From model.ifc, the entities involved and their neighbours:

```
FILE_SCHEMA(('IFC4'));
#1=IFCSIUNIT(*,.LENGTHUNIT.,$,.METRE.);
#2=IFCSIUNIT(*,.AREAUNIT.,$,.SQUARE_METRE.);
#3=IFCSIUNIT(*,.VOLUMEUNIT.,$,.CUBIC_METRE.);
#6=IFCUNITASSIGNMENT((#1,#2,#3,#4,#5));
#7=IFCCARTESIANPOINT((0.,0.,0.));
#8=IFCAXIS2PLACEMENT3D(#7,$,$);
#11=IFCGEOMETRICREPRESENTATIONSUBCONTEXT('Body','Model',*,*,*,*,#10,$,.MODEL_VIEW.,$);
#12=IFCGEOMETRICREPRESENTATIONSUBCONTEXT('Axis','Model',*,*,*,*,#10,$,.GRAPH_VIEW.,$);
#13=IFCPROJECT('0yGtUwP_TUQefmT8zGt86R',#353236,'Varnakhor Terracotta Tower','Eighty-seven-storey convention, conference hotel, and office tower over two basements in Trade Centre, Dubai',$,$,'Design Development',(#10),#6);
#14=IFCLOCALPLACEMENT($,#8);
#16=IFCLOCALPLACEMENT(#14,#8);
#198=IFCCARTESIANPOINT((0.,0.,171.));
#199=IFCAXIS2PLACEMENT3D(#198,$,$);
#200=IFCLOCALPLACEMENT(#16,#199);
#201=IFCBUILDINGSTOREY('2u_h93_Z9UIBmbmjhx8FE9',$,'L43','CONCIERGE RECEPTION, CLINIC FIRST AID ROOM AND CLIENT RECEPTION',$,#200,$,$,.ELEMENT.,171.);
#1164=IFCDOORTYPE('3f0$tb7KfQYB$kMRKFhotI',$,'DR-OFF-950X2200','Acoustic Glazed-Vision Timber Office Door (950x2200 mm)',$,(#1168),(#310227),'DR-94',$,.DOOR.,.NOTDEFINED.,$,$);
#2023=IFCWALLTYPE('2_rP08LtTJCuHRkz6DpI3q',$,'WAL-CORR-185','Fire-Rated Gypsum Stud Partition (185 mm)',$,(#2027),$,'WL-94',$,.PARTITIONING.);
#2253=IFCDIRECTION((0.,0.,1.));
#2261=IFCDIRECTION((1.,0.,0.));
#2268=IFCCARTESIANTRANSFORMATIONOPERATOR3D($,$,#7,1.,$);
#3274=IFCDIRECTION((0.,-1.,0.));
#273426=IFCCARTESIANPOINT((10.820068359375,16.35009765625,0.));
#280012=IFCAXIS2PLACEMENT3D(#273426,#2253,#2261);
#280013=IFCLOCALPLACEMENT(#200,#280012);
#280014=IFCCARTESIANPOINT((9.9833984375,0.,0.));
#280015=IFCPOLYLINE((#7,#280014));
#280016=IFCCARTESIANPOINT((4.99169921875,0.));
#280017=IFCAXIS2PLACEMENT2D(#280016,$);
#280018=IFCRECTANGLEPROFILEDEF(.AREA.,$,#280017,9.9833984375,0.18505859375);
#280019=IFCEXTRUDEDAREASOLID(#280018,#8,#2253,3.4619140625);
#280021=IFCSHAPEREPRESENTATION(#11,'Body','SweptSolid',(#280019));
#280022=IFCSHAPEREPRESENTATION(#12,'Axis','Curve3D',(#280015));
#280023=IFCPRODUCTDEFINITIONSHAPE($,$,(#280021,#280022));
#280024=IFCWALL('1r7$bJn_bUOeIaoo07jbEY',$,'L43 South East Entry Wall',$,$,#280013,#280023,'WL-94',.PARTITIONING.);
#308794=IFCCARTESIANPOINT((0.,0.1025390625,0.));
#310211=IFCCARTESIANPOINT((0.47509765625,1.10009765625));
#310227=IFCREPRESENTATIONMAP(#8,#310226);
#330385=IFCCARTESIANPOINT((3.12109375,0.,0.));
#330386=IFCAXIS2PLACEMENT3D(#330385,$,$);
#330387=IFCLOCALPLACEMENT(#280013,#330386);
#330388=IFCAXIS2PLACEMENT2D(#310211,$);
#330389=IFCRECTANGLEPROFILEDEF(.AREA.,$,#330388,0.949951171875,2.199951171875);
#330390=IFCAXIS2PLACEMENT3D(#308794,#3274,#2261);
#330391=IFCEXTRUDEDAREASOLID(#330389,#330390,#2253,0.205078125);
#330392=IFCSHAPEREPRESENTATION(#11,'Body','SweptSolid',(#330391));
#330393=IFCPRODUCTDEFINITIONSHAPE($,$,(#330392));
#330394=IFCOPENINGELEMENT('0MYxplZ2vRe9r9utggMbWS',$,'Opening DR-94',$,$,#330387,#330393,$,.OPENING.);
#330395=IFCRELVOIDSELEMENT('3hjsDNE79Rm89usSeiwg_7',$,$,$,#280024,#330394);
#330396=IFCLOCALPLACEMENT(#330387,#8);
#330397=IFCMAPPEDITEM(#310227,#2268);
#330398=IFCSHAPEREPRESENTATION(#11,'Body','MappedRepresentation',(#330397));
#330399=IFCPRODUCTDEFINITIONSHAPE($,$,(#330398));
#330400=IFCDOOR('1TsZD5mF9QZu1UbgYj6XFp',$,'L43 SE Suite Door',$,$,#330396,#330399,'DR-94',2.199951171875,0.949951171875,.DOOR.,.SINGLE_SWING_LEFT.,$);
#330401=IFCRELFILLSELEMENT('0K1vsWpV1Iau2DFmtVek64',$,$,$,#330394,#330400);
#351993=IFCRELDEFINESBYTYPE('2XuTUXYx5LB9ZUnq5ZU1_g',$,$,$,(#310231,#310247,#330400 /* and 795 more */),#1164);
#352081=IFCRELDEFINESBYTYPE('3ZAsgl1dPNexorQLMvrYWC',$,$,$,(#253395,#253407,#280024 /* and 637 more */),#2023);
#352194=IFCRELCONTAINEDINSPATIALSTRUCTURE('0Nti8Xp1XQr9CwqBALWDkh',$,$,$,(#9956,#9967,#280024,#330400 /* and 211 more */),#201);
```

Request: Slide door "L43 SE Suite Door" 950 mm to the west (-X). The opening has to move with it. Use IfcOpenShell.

```python
import ifcopenshell
import ifcopenshell.api.geometry
import ifcopenshell.util.placement
import ifcopenshell.util.unit

model = ifcopenshell.open("model.ifc")
unit_scale = ifcopenshell.util.unit.calculate_unit_scale(model)

door = model.by_guid("1TsZD5mF9QZu1UbgYj6XFp")
opening = door.FillsVoids[0].RelatingOpeningElement
wall = opening.VoidsElements[0].RelatingBuildingElement

wall_matrix = ifcopenshell.util.placement.get_local_placement(wall.ObjectPlacement)
shift = wall_matrix[:3, 0] * -0.95 / unit_scale
before = ifcopenshell.util.placement.get_local_placement(door.ObjectPlacement)[:3, 3].copy()

# The door is placed relative to its opening, so it follows when the opening moves.
matrix = ifcopenshell.util.placement.get_local_placement(opening.ObjectPlacement)
matrix[:3, 3] += shift
ifcopenshell.api.geometry.edit_object_placement(
    model, product=opening, matrix=matrix, is_si=False, should_transform_children=True
)

after = ifcopenshell.util.placement.get_local_placement(door.ObjectPlacement)[:3, 3]
print("door moved by", (after - before).round(3) + 0.0)

model.write("model_rev.ifc")
```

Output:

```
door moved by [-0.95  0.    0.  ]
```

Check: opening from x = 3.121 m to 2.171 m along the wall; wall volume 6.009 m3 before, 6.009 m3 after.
